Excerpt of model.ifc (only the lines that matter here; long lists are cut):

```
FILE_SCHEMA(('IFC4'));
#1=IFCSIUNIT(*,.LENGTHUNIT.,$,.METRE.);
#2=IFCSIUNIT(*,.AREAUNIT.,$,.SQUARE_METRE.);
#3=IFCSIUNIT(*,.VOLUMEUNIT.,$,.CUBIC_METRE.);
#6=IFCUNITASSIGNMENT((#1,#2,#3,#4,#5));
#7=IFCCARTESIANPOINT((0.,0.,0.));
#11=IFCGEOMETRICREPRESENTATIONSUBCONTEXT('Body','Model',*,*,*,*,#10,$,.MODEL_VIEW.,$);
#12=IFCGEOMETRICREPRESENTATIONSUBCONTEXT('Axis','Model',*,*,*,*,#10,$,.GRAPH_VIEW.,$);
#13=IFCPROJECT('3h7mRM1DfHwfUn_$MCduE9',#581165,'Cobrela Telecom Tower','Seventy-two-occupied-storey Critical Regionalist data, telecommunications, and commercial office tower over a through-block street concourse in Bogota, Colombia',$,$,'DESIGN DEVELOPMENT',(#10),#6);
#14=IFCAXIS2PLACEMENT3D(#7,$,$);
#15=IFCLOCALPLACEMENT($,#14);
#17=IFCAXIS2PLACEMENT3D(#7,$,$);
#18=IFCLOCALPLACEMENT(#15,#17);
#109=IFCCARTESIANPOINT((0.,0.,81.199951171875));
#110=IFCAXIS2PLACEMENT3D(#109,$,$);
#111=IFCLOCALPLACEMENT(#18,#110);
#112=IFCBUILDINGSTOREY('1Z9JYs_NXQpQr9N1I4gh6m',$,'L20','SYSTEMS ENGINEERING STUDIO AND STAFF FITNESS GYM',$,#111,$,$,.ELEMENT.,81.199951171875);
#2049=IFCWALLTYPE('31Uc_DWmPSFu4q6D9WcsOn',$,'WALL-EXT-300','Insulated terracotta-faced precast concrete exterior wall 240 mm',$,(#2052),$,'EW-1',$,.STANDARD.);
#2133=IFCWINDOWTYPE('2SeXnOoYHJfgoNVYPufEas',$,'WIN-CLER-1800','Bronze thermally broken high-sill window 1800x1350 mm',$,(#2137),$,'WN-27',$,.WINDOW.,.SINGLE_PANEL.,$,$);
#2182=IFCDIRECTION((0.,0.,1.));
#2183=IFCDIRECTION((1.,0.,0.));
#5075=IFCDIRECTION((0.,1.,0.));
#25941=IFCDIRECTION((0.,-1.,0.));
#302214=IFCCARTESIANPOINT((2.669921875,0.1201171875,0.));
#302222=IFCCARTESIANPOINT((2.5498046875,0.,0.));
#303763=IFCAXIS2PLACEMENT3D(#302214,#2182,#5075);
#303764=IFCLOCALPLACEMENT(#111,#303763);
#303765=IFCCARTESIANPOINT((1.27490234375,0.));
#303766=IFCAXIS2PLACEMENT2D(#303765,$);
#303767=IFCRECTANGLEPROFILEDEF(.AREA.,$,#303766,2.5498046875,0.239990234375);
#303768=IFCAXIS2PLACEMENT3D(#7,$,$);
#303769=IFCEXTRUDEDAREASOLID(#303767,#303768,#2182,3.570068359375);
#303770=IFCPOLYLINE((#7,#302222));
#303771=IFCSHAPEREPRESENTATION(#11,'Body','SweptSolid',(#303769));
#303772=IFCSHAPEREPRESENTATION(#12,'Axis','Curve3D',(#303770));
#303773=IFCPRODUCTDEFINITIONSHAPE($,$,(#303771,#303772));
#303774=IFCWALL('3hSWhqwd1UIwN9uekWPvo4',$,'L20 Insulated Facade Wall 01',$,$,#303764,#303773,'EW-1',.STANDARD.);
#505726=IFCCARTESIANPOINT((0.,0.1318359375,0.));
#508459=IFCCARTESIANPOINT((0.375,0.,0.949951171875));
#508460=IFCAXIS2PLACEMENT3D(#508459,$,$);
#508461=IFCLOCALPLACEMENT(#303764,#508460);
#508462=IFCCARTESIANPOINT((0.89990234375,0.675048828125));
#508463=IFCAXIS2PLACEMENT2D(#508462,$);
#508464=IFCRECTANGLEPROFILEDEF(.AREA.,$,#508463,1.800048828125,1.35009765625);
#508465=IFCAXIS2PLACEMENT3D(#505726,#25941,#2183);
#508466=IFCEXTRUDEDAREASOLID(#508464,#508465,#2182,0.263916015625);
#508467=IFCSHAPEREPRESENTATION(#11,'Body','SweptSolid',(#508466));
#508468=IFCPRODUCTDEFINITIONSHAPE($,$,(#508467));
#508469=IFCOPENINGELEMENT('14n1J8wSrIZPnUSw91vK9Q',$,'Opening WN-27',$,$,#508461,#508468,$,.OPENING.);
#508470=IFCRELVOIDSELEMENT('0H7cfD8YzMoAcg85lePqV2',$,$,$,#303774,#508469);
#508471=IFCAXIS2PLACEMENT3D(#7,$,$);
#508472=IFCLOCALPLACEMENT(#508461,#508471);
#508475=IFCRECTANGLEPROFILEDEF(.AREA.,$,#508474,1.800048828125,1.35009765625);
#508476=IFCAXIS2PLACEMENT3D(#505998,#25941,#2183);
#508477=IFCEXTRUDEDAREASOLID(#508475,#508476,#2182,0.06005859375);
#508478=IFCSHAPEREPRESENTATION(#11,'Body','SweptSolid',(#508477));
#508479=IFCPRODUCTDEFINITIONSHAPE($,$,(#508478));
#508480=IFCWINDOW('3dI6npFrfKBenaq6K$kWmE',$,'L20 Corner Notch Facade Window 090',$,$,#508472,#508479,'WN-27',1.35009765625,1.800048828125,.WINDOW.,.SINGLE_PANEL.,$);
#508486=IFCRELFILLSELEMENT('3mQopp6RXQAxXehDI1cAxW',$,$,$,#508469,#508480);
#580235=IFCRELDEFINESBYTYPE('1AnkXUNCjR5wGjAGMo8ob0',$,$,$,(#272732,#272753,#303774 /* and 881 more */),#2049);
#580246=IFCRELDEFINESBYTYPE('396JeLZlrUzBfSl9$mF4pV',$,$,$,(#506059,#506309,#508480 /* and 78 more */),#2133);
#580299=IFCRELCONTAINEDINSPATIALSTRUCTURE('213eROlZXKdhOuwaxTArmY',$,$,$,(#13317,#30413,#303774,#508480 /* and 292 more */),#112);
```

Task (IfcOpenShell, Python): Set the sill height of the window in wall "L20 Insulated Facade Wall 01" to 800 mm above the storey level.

```python
import numpy as np
import ifcopenshell
import ifcopenshell.api.geometry
import ifcopenshell.geom
import ifcopenshell.util.element
import ifcopenshell.util.placement
import ifcopenshell.util.shape
import ifcopenshell.util.unit

model = ifcopenshell.open("model.ifc")
unit_scale = ifcopenshell.util.unit.calculate_unit_scale(model)

window = model.by_id(508480)
opening = window.FillsVoids[0].RelatingOpeningElement
storey = ifcopenshell.util.element.get_container(window, ifc_class="IfcBuildingStorey")
level = ifcopenshell.util.placement.get_local_placement(storey.ObjectPlacement)[2, 3]

# The opening's origin need not be at the sill, so measure its lowest point.
shape = ifcopenshell.geom.create_shape(ifcopenshell.geom.settings(), opening)
bottom = ifcopenshell.util.shape.get_shape_bottom_elevation(shape, shape.geometry) / unit_scale
dz = level + 0.8 - bottom

shift = np.array([0.0, 0.0, dz])
# The window is placed relative to its opening, so it follows when the opening moves.
matrix = ifcopenshell.util.placement.get_local_placement(opening.ObjectPlacement)
matrix[:3, 3] += shift
ifcopenshell.api.geometry.edit_object_placement(
    model, product=opening, matrix=matrix, is_si=False, should_transform_children=True
)

print(f"moved by {dz * unit_scale:+.3f} m")

model.write("model_updated.ifc")
```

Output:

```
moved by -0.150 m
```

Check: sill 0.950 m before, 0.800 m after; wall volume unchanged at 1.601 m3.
